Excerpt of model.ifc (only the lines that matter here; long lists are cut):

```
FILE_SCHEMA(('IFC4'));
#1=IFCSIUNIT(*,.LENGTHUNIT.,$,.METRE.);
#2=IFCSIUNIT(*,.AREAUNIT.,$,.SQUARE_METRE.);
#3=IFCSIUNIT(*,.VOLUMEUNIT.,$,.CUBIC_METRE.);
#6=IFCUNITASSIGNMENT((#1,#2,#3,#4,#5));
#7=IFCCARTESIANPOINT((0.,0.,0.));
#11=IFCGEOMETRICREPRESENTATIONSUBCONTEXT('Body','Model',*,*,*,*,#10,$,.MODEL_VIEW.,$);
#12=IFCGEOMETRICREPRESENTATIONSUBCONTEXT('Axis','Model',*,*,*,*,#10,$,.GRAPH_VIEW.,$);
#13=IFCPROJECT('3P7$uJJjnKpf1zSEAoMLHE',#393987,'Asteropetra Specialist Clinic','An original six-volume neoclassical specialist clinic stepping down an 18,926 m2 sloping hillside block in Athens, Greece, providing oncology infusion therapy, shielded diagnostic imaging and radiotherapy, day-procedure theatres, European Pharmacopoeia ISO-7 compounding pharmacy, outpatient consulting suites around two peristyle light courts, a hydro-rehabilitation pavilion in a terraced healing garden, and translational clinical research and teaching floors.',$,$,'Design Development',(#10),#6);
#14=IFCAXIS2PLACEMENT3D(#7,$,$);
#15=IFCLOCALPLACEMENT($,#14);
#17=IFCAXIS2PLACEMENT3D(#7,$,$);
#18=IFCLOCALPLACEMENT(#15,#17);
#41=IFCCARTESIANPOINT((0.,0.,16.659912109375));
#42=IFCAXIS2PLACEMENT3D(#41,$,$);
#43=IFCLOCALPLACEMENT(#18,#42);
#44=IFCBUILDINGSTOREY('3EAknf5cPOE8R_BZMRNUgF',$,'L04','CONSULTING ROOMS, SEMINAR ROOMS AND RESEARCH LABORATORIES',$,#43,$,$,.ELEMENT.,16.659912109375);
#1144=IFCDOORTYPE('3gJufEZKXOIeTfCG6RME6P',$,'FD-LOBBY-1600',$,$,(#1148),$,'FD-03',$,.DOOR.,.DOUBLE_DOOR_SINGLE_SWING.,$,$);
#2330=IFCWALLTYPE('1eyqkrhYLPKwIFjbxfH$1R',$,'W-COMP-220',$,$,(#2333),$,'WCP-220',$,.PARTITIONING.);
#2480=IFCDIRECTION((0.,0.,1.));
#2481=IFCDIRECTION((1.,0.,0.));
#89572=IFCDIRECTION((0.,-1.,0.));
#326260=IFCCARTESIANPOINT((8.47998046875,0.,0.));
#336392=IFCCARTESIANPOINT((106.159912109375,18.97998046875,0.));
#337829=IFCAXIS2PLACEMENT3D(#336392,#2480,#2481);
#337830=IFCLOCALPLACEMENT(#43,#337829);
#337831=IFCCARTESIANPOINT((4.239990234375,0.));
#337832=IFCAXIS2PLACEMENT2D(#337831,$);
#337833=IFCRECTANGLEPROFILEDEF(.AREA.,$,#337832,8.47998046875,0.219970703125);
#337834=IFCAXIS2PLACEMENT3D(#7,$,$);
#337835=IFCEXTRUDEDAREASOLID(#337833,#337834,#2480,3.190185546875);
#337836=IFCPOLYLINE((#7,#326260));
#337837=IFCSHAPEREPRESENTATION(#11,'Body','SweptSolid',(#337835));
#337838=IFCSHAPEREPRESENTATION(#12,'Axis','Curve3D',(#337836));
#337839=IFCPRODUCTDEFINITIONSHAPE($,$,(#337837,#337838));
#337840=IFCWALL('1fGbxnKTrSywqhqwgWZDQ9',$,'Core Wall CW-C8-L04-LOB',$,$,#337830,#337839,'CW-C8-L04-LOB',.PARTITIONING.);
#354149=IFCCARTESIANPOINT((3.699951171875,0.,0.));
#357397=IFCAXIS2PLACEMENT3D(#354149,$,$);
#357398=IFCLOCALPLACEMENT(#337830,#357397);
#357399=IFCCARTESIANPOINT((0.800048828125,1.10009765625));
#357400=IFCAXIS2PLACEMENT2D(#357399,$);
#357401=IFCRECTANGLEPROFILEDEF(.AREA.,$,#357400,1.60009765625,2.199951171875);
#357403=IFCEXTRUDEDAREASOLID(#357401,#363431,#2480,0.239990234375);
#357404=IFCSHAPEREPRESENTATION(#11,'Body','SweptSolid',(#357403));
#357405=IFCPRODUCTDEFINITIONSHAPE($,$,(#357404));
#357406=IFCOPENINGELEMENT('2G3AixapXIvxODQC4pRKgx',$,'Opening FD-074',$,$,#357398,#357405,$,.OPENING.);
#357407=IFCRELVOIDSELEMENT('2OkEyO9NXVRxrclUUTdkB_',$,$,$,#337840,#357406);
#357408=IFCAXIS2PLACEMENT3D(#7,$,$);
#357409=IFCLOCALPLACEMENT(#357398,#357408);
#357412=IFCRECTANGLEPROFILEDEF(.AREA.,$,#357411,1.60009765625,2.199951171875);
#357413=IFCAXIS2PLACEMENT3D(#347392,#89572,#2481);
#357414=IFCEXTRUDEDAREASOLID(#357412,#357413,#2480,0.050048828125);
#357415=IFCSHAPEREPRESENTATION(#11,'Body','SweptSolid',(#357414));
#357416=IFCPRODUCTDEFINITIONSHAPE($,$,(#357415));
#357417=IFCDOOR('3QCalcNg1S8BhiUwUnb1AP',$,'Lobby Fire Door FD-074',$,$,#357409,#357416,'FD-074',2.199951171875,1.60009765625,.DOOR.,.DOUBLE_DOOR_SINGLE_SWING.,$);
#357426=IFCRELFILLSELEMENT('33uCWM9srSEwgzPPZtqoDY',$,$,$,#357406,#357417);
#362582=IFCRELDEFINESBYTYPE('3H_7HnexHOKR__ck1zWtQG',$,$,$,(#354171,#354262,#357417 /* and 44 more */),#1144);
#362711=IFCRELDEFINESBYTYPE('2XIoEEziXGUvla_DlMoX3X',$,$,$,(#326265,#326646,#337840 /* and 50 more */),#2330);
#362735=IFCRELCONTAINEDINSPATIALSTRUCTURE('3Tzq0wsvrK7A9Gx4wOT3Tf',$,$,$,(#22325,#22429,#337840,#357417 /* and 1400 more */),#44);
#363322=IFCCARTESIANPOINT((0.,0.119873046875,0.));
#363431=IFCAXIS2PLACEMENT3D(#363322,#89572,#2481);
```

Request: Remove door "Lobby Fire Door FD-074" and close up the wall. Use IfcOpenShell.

```python
import ifcopenshell
import ifcopenshell.api.feature
import ifcopenshell.api.root
import ifcopenshell.geom
import ifcopenshell.util.shape

model = ifcopenshell.open("model.ifc")
settings = ifcopenshell.geom.settings()


def volume(element):
    """Net volume in cubic metres, openings subtracted."""
    shape = ifcopenshell.geom.create_shape(settings, element)
    return ifcopenshell.util.shape.get_volume(shape.geometry)


door = model.by_guid("3QCalcNg1S8BhiUwUnb1AP")
opening = door.FillsVoids[0].RelatingOpeningElement
wall = opening.VoidsElements[0].RelatingBuildingElement
before = volume(wall)

ifcopenshell.api.root.remove_product(model, product=door)
ifcopenshell.api.feature.remove_feature(model, feature=opening)

after = volume(wall)

print(f"wall volume {before:.3f} -> {after:.3f} m3")

model.write("model_edited.ifc")
```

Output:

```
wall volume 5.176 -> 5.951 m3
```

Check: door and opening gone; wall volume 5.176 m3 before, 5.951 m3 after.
